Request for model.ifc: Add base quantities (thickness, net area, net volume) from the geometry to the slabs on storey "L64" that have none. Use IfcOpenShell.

First a look at what the model holds.

```python
import ifcopenshell
import ifcopenshell.util.element
import ifcopenshell.util.unit

model = ifcopenshell.open("model.ifc")
print(model.schema)
for unit_type in ("LENGTHUNIT", "AREAUNIT", "VOLUMEUNIT"):
    print(unit_type, ifcopenshell.util.unit.calculate_unit_scale(model, unit_type))
storey = next(s for s in model.by_type("IfcBuildingStorey") if s.Name == "L64")
slabs = [e for e in ifcopenshell.util.element.get_decomposition(storey) if e.is_a("IfcSlab")]
for e in sorted(slabs, key=lambda e: e.id()):
    print(e.id(), e.is_a(), e.Name, list(ifcopenshell.util.element.get_psets(e, qtos_only=True)), sep=" | ")
```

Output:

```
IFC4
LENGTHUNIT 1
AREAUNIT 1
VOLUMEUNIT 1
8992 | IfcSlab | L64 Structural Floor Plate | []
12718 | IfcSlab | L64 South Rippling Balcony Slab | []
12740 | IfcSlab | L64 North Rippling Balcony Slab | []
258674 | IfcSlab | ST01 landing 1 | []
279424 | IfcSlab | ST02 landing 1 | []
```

```python
import ifcopenshell
import ifcopenshell.api.pset
import ifcopenshell.geom
import ifcopenshell.util.element
import ifcopenshell.util.shape
import ifcopenshell.util.unit

model = ifcopenshell.open("model.ifc")
unit_scale = ifcopenshell.util.unit.calculate_unit_scale(model)
area_scale = ifcopenshell.util.unit.calculate_unit_scale(model, "AREAUNIT")
volume_scale = ifcopenshell.util.unit.calculate_unit_scale(model, "VOLUMEUNIT")
settings = ifcopenshell.geom.settings()

storey = next(s for s in model.by_type("IfcBuildingStorey") if s.Name == "L64")
slabs = [e for e in ifcopenshell.util.element.get_decomposition(storey) if e.is_a("IfcSlab")]

for e in sorted(slabs, key=lambda e: e.id()):
    if ifcopenshell.util.element.get_psets(e, qtos_only=True, should_inherit=False):
        continue
    # Geometry comes back in metres, in the element's own axes.
    shape = ifcopenshell.geom.create_shape(settings, e)
    values = {
        "Width": ifcopenshell.util.shape.get_z(shape.geometry) / unit_scale,
        "NetArea": ifcopenshell.util.shape.get_footprint_area(shape.geometry) / area_scale,
        "NetVolume": ifcopenshell.util.shape.get_volume(shape.geometry) / volume_scale,
    }
    qto = ifcopenshell.api.pset.add_qto(model, product=e, name="Qto_SlabBaseQuantities")
    ifcopenshell.api.pset.edit_qto(model, qto=qto, properties=values)
    print(e.id(), {k: round(v, 3) for k, v in values.items()})

model.write("model_v2.ifc")
```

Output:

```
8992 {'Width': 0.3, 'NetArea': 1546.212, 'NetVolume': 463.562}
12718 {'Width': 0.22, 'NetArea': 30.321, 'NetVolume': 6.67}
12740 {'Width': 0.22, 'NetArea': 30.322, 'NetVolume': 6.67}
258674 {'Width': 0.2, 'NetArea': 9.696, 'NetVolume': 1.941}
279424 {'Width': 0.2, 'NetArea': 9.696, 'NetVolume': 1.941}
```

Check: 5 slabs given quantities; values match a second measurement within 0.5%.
